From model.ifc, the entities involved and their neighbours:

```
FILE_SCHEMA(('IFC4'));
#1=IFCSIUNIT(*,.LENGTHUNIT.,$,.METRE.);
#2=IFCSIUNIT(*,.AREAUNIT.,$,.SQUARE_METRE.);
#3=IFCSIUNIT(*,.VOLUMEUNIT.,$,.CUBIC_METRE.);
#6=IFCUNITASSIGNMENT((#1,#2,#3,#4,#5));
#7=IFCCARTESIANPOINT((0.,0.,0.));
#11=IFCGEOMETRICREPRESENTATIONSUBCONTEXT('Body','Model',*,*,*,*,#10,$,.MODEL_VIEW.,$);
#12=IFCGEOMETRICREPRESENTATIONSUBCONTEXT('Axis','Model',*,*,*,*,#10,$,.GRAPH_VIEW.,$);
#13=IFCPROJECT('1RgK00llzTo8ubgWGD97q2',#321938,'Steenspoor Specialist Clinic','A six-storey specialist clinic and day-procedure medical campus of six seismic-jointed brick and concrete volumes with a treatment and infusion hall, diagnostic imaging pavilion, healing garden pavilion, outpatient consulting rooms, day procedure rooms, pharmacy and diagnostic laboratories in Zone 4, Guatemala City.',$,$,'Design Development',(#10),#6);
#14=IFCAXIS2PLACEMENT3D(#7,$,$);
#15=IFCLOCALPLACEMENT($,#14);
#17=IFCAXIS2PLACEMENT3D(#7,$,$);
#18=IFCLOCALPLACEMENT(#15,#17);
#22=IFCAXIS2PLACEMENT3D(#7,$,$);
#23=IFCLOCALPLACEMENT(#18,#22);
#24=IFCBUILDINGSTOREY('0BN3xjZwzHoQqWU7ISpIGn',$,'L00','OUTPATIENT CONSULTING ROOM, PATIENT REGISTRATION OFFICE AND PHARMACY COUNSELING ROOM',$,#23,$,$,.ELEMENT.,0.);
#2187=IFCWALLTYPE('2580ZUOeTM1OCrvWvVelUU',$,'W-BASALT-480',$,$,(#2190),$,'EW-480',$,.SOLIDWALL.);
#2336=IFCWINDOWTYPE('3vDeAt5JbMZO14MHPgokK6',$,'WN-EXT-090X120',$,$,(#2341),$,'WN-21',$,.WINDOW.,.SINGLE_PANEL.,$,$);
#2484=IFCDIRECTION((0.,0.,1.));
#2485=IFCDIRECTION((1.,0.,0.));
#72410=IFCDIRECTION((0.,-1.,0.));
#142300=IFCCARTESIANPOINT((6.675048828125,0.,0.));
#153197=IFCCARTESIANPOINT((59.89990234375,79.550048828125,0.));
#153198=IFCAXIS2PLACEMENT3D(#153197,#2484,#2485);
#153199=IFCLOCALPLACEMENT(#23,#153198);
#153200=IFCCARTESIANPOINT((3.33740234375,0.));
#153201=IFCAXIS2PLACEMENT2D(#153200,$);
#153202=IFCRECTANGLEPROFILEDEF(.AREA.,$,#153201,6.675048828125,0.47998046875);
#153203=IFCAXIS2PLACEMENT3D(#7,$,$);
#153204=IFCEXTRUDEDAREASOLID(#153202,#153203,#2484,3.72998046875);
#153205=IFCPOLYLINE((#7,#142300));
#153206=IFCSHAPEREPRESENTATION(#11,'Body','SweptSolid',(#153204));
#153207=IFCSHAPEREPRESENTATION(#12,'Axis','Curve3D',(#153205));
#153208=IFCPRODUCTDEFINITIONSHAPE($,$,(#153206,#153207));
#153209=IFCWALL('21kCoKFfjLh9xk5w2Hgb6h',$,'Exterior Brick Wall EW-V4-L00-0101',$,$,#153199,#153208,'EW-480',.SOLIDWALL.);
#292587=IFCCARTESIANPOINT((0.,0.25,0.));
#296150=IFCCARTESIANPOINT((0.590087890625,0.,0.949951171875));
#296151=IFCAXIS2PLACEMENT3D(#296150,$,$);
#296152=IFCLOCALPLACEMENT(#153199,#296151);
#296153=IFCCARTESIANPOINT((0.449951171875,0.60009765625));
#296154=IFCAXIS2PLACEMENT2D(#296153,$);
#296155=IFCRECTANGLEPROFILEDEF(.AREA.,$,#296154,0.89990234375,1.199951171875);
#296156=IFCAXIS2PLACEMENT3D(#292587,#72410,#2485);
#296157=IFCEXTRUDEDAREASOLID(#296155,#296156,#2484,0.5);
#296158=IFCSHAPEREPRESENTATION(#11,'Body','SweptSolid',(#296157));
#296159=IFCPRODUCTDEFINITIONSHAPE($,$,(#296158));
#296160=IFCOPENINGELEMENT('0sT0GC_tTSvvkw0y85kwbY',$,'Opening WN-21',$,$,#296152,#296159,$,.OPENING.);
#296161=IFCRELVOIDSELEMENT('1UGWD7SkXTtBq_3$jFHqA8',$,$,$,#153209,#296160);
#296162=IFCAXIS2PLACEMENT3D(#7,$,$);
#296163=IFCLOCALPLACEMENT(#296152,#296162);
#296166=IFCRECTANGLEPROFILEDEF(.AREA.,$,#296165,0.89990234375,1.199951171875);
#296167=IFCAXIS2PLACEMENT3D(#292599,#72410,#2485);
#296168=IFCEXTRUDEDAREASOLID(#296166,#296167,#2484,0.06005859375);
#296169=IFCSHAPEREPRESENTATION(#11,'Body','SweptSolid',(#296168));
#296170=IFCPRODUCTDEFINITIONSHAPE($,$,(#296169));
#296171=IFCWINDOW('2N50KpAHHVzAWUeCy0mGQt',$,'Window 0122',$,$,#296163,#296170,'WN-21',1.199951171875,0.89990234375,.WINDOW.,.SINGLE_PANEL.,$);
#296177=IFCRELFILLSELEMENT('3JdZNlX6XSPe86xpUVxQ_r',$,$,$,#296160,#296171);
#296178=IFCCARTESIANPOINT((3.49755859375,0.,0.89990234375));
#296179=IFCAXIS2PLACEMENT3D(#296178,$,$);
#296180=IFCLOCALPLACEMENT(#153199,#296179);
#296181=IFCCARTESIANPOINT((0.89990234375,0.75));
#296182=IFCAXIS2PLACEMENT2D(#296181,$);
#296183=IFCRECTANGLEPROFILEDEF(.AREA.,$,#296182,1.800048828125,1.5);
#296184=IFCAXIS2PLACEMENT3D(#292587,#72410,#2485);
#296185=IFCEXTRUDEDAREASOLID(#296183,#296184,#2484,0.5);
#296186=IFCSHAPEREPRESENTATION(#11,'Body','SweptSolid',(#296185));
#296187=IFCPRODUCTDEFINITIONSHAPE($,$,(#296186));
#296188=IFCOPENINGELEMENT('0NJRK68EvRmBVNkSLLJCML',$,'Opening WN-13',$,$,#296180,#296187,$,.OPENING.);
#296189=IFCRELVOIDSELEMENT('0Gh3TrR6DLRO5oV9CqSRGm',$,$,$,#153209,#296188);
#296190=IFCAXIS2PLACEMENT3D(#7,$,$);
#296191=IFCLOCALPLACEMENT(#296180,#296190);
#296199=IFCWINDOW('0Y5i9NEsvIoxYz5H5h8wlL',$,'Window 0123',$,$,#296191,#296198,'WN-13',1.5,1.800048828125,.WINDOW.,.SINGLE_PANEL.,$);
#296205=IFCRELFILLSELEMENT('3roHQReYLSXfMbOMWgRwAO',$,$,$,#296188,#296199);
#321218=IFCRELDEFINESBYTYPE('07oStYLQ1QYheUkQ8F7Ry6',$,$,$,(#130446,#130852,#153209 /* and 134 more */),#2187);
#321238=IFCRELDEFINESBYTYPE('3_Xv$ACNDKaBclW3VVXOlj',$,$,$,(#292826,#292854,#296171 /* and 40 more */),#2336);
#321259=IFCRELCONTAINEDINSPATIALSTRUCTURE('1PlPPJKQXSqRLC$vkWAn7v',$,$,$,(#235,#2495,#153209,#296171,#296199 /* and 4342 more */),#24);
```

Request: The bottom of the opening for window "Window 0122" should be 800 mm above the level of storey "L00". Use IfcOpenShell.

```python
import numpy as np
import ifcopenshell
import ifcopenshell.api.geometry
import ifcopenshell.geom
import ifcopenshell.util.element
import ifcopenshell.util.placement
import ifcopenshell.util.shape
import ifcopenshell.util.unit

model = ifcopenshell.open("model.ifc")
unit_scale = ifcopenshell.util.unit.calculate_unit_scale(model)

window = model.by_guid("2N50KpAHHVzAWUeCy0mGQt")
opening = window.FillsVoids[0].RelatingOpeningElement
storey = ifcopenshell.util.element.get_container(window, ifc_class="IfcBuildingStorey")
level = ifcopenshell.util.placement.get_local_placement(storey.ObjectPlacement)[2, 3]

# The opening's origin need not be at the sill, so measure its lowest point.
shape = ifcopenshell.geom.create_shape(ifcopenshell.geom.settings(), opening)
bottom = ifcopenshell.util.shape.get_shape_bottom_elevation(shape, shape.geometry) / unit_scale
dz = level + 0.8 / unit_scale - bottom

shift = np.array([0.0, 0.0, dz])
# The window is placed relative to its opening, so it follows when the opening moves.
matrix = ifcopenshell.util.placement.get_local_placement(opening.ObjectPlacement)
matrix[:3, 3] += shift
ifcopenshell.api.geometry.edit_object_placement(
    model, product=opening, matrix=matrix, is_si=False, should_transform_children=True
)

print(f"moved by {dz * unit_scale:+.3f} m")

model.write("model-out.ifc")
```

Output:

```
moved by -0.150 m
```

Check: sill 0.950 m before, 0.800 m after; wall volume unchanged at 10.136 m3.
